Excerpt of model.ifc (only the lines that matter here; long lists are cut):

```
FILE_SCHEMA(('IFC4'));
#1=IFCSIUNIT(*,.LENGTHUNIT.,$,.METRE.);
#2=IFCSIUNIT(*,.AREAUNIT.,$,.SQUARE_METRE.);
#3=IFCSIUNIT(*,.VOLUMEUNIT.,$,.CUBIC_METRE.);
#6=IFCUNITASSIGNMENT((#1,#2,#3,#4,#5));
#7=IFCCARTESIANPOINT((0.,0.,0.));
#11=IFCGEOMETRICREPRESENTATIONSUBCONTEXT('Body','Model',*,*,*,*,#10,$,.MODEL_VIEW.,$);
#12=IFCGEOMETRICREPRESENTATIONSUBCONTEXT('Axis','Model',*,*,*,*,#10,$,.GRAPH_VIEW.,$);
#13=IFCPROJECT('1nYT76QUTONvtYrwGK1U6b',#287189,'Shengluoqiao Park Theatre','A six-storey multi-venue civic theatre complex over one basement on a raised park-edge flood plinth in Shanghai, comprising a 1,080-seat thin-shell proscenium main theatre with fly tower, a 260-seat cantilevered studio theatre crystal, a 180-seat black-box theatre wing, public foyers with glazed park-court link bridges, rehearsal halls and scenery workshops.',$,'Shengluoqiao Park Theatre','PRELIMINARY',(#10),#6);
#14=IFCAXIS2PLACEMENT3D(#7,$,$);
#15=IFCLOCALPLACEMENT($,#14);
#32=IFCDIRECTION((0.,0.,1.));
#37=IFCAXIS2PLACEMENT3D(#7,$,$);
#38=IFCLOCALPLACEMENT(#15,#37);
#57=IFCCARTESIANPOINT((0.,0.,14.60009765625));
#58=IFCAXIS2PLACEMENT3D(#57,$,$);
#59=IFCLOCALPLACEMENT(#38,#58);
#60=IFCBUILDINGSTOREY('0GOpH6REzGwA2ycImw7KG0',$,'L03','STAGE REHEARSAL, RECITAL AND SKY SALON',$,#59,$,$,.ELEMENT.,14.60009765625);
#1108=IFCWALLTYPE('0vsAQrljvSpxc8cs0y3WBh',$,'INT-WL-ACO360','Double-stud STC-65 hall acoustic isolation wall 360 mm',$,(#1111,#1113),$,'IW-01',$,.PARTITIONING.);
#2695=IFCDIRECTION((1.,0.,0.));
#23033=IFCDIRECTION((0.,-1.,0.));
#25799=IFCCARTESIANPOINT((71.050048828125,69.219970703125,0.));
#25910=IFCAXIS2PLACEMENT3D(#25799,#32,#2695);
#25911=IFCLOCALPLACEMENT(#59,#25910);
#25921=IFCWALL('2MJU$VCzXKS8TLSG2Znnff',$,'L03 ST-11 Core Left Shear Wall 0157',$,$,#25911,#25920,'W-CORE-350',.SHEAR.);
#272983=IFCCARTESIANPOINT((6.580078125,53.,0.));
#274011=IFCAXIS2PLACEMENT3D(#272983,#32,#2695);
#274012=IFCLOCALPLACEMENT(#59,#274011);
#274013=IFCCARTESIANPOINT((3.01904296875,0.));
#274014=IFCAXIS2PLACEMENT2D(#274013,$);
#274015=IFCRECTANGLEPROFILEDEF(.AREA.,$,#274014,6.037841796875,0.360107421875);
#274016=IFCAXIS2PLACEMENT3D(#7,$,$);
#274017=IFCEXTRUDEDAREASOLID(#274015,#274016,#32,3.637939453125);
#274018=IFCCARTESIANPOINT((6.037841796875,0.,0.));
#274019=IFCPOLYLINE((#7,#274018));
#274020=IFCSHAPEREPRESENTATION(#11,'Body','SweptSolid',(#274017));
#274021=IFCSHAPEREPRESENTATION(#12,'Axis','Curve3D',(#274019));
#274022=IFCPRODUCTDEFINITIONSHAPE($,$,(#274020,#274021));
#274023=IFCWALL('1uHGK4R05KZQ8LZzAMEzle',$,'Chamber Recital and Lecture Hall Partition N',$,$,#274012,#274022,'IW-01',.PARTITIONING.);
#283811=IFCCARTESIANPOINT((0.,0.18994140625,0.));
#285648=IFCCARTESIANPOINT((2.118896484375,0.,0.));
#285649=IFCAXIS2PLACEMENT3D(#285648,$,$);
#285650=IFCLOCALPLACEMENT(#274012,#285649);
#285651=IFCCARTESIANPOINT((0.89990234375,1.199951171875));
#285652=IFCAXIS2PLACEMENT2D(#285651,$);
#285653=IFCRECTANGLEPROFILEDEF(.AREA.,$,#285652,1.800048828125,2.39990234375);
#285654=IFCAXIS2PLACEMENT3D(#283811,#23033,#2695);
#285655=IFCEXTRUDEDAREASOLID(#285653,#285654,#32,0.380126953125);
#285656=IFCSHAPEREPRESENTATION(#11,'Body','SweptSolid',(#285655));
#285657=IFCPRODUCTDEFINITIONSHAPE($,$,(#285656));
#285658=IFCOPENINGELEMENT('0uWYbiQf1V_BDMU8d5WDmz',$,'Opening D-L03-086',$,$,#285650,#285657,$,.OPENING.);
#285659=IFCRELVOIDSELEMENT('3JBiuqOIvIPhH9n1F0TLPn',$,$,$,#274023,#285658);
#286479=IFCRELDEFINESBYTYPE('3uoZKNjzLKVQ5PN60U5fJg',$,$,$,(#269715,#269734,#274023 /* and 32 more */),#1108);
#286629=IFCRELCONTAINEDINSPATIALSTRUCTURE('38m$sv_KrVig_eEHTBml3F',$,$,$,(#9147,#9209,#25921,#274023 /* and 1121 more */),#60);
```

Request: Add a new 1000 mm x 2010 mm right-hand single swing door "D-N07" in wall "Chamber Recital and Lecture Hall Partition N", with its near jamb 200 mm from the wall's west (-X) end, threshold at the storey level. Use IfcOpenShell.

```python
import numpy as np
import ifcopenshell
import ifcopenshell.api.feature
import ifcopenshell.api.geometry
import ifcopenshell.api.root
import ifcopenshell.api.spatial
import ifcopenshell.geom
import ifcopenshell.util.element
import ifcopenshell.util.placement
import ifcopenshell.util.representation
import ifcopenshell.util.shape
import ifcopenshell.util.unit

model = ifcopenshell.open("model.ifc")
unit_scale = ifcopenshell.util.unit.calculate_unit_scale(model)
settings = ifcopenshell.geom.settings()


def volume(element):
    """Net volume in cubic metres, openings subtracted."""
    shape = ifcopenshell.geom.create_shape(settings, element)
    return ifcopenshell.util.shape.get_volume(shape.geometry)


wall = model.by_id(274023)
storey = ifcopenshell.util.element.get_container(wall, ifc_class="IfcBuildingStorey")
context = ifcopenshell.util.representation.get_context(model, "Model", "Body", "MODEL_VIEW")
before = volume(wall)

width, height, from_end, sill = 1, 2.01, 0.2, 0.0  # metres

# The wall runs along its own X axis, and the end named is its -X end.
wall_shape = ifcopenshell.geom.create_shape(settings, wall)
x, y, z = ifcopenshell.util.shape.get_vertices(wall_shape.geometry).T
start = x.min() + from_end
face, thickness = float(y.min()), float(y.max() - y.min())
wall_matrix = ifcopenshell.util.placement.get_local_placement(wall.ObjectPlacement)
level = ifcopenshell.util.placement.get_local_placement(storey.ObjectPlacement)[2, 3]


def in_wall(x, y):
    """Placement at x, y metres in the wall's axes, at sill height."""
    matrix = wall_matrix.copy()
    matrix[:, 3] = wall_matrix @ np.array([x / unit_scale, y / unit_scale, 0.0, 1.0])
    matrix[2, 3] = level + sill / unit_scale
    return matrix


# Opening: a box that overshoots both wall faces by 50 mm.
opening = ifcopenshell.api.root.create_entity(model, ifc_class="IfcOpeningElement", predefined_type="OPENING")
box = ifcopenshell.api.geometry.add_wall_representation(
    model, context=context, length=width, height=height, thickness=thickness + 0.1
)
ifcopenshell.api.geometry.assign_representation(model, product=opening, representation=box)
ifcopenshell.api.geometry.edit_object_placement(model, product=opening, matrix=in_wall(start, face - 0.05), is_si=False)
ifcopenshell.api.feature.add_feature(model, feature=opening, element=wall)

door = ifcopenshell.api.root.create_entity(model, ifc_class="IfcDoor", name="D-N07", predefined_type="DOOR")
door.OverallWidth, door.OverallHeight = width / unit_scale, height / unit_scale
door.OperationType = "SINGLE_SWING_RIGHT"
body = ifcopenshell.api.geometry.add_door_representation(
    model,
    context=context,
    overall_width=door.OverallWidth,
    overall_height=door.OverallHeight,
    operation_type="SINGLE_SWING_RIGHT",
    lining_properties={"LiningDepth": thickness / unit_scale, "ThresholdDepth": thickness / unit_scale},
)
ifcopenshell.api.geometry.assign_representation(model, product=door, representation=body)
ifcopenshell.api.spatial.assign_container(model, products=[door], relating_structure=storey)
ifcopenshell.api.feature.add_filling(model, opening=opening, element=door)

# The lining spans the wall, so the door starts at the wall face.
ifcopenshell.api.geometry.edit_object_placement(model, product=door, matrix=in_wall(start, face), is_si=False)

after = volume(wall)

print(f"wall volume {before:.3f} -> {after:.3f} m3")

model.write("model_edited.ifc")
```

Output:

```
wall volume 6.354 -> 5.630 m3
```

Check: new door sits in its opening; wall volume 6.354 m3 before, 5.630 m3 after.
